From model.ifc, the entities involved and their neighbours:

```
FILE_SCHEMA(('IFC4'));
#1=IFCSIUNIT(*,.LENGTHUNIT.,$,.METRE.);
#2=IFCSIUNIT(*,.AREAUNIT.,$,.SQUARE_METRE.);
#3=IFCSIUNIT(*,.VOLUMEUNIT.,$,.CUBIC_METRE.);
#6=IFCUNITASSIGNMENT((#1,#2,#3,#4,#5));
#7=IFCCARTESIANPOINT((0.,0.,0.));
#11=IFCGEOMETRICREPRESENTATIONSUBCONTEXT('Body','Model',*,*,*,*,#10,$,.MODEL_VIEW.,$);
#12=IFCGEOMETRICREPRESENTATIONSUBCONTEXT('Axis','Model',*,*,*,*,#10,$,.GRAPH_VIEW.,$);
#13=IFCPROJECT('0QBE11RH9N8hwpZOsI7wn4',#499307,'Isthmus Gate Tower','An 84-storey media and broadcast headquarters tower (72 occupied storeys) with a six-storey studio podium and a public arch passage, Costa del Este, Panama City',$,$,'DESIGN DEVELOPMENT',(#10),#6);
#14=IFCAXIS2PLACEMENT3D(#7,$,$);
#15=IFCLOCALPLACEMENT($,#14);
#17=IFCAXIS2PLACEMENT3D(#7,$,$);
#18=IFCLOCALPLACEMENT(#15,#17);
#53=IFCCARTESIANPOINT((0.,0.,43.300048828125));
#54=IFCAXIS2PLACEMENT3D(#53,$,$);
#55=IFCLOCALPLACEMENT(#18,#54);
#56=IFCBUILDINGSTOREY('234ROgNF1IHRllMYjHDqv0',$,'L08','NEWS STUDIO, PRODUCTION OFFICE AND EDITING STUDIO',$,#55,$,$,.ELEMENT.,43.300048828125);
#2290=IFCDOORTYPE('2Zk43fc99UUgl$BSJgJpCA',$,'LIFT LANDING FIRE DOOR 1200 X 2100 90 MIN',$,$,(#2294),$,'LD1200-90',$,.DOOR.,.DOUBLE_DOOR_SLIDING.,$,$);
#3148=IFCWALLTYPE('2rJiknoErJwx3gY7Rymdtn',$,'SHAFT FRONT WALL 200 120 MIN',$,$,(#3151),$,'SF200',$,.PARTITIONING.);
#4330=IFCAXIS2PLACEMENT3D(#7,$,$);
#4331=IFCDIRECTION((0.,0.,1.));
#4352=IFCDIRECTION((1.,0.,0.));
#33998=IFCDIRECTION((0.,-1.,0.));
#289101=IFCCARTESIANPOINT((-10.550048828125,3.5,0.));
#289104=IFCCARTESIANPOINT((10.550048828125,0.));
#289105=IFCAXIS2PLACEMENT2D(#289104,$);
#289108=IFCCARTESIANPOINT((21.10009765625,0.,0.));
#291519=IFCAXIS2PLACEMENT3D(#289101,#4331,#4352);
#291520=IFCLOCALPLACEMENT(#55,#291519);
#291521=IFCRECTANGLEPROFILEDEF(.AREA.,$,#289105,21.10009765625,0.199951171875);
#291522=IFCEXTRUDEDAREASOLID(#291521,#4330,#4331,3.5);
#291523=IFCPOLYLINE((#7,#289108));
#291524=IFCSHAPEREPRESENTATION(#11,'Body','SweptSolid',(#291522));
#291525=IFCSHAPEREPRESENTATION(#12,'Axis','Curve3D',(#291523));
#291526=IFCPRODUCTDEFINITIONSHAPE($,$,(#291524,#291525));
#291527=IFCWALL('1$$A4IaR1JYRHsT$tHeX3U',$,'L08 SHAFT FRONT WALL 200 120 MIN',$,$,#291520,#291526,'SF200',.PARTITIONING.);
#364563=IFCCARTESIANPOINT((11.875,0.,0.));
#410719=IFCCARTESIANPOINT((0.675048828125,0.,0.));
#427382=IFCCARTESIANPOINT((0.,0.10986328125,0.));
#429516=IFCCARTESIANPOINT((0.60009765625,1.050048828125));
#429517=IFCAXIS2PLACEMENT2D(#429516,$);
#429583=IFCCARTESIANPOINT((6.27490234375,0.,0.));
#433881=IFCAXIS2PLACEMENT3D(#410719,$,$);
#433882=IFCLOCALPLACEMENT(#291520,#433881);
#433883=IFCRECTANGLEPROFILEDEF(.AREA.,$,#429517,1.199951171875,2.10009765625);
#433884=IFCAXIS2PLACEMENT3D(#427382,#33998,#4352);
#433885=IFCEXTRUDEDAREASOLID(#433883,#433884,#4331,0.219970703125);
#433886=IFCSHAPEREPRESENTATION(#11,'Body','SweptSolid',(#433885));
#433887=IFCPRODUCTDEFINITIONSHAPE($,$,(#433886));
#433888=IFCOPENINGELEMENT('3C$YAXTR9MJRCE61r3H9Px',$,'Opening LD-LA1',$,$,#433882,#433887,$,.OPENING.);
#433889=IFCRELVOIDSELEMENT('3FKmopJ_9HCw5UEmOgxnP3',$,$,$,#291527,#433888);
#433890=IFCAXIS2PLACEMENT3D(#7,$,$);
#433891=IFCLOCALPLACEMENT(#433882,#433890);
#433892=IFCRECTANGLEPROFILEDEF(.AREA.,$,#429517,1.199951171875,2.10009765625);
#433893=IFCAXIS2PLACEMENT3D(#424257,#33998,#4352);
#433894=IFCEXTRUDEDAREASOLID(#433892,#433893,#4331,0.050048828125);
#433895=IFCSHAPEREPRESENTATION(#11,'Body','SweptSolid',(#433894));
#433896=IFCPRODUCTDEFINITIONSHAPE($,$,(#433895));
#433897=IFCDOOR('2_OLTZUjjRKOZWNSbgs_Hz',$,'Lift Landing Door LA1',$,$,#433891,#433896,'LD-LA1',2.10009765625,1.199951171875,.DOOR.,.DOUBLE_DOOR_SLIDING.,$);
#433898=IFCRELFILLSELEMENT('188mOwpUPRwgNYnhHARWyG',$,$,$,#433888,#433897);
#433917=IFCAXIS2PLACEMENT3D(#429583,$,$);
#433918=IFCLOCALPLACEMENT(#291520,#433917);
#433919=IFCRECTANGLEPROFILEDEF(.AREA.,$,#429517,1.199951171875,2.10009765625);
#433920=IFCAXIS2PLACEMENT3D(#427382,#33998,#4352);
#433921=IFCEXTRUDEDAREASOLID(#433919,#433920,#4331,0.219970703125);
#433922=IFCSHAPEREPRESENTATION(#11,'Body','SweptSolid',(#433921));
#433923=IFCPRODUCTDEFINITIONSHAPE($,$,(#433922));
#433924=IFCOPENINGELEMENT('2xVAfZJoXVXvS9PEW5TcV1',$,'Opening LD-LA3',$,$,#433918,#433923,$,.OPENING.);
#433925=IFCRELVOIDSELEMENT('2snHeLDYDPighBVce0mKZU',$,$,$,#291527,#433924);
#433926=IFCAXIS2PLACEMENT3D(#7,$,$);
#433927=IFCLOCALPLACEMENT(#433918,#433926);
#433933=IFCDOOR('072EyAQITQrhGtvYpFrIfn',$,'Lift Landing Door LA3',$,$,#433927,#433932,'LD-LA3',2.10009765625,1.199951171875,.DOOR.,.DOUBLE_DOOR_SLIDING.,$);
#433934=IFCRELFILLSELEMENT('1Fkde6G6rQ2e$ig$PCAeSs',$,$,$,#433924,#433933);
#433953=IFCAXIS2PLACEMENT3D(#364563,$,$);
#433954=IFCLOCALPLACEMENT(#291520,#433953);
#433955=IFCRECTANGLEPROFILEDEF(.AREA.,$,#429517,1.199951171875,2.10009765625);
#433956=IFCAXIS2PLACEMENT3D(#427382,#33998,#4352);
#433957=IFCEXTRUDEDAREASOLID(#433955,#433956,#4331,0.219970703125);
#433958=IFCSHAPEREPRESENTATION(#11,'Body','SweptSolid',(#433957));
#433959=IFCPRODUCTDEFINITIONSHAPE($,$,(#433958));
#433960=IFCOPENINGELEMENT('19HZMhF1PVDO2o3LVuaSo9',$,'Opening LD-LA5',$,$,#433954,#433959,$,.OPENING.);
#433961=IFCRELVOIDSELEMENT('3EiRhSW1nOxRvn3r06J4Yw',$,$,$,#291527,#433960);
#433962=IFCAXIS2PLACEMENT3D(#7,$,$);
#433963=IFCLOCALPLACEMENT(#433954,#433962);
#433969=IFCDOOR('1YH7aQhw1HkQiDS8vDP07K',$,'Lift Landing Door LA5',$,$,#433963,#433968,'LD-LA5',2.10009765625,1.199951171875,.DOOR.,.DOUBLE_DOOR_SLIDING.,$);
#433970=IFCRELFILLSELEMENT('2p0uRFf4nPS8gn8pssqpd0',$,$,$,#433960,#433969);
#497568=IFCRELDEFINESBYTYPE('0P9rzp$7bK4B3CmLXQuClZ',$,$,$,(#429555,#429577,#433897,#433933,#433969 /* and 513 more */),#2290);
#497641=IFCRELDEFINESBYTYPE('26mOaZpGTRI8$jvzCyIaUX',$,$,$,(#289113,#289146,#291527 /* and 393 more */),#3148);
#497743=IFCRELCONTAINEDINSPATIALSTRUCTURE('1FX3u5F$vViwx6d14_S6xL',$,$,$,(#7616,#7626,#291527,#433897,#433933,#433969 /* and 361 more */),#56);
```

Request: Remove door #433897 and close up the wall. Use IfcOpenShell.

```python
import ifcopenshell
import ifcopenshell.api.feature
import ifcopenshell.api.root
import ifcopenshell.geom
import ifcopenshell.util.shape

model = ifcopenshell.open("model.ifc")
settings = ifcopenshell.geom.settings()


def volume(element):
    """Net volume in cubic metres, openings subtracted."""
    shape = ifcopenshell.geom.create_shape(settings, element)
    return ifcopenshell.util.shape.get_volume(shape.geometry)


door = model.by_guid("2_OLTZUjjRKOZWNSbgs_Hz")
opening = door.FillsVoids[0].RelatingOpeningElement
wall = opening.VoidsElements[0].RelatingBuildingElement
before = volume(wall)

ifcopenshell.api.root.remove_product(model, product=door)
ifcopenshell.api.feature.remove_feature(model, feature=opening)

after = volume(wall)

print(f"wall volume {before:.3f} -> {after:.3f} m3")

model.write("model_edited.ifc")
```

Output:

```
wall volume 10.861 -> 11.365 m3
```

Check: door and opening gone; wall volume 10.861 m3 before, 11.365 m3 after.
